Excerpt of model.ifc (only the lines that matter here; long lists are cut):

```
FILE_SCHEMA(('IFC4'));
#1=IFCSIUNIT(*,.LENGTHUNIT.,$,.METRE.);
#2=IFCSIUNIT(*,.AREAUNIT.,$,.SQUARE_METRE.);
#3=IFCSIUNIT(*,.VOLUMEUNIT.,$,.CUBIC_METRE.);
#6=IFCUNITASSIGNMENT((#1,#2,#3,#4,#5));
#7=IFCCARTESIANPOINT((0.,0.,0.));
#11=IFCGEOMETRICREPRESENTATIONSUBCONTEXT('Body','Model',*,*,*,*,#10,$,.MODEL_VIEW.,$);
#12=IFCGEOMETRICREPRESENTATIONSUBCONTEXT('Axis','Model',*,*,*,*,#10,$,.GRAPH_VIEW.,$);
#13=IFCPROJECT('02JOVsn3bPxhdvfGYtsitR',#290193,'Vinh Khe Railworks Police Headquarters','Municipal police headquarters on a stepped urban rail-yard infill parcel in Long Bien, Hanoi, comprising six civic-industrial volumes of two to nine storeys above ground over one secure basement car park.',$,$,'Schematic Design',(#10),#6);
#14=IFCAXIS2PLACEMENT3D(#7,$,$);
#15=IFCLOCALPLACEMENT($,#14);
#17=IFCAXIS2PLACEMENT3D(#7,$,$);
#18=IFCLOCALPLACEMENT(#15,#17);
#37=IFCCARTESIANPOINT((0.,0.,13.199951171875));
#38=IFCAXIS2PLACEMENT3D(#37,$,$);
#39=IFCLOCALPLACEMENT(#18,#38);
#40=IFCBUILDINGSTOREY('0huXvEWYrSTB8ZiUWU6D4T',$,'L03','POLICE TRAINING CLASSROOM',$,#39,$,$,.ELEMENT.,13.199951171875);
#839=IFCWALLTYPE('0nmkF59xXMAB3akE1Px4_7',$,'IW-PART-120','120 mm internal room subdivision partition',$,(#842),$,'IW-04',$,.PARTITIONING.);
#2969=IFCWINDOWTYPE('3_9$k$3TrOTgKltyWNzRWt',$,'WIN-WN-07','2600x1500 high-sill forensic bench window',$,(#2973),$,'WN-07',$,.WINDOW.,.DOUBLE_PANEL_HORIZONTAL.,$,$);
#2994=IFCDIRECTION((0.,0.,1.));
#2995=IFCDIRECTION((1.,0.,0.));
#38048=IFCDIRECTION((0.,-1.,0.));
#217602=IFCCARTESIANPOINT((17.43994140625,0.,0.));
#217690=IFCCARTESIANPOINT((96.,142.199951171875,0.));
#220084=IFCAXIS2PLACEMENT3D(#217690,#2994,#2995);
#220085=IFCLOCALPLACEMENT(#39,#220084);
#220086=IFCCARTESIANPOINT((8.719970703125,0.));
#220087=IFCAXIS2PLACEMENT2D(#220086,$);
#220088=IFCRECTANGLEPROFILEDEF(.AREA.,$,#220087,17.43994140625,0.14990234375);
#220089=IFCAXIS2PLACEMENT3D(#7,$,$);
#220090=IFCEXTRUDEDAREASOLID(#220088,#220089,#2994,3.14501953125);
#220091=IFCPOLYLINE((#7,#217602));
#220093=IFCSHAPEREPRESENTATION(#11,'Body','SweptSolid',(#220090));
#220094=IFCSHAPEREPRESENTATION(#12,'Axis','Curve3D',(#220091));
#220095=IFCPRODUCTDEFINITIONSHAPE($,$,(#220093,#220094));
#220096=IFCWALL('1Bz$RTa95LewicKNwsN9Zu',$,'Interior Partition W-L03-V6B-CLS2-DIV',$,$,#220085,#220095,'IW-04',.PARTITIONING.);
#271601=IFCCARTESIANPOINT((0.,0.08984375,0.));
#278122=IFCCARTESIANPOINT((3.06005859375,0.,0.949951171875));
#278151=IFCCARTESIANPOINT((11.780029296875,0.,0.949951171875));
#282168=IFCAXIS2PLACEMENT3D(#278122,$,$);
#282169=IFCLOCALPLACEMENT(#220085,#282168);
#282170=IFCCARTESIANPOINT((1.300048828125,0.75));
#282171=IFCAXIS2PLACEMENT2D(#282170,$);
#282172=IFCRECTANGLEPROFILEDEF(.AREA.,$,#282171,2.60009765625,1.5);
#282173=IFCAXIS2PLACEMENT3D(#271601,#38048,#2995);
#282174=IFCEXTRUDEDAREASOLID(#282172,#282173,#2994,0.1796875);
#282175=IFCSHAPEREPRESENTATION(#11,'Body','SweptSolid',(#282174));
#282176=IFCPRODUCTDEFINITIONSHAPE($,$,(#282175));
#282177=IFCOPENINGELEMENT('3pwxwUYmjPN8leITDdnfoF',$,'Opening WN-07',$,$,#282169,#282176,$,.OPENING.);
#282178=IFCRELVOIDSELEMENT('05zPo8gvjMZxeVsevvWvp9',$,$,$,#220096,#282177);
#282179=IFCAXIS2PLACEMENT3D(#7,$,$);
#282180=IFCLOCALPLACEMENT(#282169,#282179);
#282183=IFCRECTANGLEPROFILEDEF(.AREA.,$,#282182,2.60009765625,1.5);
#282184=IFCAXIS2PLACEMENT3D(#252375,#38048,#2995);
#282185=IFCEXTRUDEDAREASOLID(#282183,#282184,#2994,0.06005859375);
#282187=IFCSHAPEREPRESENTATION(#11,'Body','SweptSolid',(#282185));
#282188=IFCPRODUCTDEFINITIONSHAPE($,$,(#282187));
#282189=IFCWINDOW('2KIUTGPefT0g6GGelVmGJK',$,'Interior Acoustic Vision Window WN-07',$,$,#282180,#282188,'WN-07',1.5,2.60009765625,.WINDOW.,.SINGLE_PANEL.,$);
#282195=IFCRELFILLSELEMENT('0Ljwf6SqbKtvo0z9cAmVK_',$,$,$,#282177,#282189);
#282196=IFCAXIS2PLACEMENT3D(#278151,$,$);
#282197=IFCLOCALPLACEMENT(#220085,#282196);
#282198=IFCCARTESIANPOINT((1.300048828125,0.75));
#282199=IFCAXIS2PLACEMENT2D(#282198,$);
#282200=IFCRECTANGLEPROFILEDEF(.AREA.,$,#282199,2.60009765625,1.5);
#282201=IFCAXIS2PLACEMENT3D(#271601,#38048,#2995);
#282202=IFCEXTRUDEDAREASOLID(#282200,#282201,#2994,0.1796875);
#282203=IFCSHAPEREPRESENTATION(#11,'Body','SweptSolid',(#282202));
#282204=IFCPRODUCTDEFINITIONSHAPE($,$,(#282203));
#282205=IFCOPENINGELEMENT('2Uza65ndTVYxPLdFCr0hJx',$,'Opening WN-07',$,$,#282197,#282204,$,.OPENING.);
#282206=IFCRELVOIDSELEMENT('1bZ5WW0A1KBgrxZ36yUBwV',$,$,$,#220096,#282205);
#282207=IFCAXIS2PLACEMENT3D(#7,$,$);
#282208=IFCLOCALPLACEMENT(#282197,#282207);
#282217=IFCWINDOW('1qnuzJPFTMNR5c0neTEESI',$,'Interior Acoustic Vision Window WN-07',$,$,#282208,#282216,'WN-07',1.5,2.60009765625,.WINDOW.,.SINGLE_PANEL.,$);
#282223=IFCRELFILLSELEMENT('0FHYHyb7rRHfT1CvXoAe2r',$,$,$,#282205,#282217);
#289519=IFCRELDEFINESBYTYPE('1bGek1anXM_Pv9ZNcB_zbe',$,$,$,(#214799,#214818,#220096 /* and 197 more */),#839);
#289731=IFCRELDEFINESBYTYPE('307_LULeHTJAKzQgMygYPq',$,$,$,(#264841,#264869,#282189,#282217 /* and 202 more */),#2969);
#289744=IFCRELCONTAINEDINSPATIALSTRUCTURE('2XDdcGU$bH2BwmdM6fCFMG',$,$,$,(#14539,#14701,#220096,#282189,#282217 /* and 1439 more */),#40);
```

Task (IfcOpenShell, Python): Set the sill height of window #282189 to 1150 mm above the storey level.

```python
import numpy as np
import ifcopenshell
import ifcopenshell.api.geometry
import ifcopenshell.geom
import ifcopenshell.util.element
import ifcopenshell.util.placement
import ifcopenshell.util.shape
import ifcopenshell.util.unit

model = ifcopenshell.open("model.ifc")
unit_scale = ifcopenshell.util.unit.calculate_unit_scale(model)

window = model.by_guid("2KIUTGPefT0g6GGelVmGJK")
opening = window.FillsVoids[0].RelatingOpeningElement
storey = ifcopenshell.util.element.get_container(window, ifc_class="IfcBuildingStorey")
level = ifcopenshell.util.placement.get_local_placement(storey.ObjectPlacement)[2, 3]

# The opening's origin need not be at the sill, so measure its lowest point.
shape = ifcopenshell.geom.create_shape(ifcopenshell.geom.settings(), opening)
bottom = ifcopenshell.util.shape.get_shape_bottom_elevation(shape, shape.geometry) / unit_scale
dz = level + 1.15 / unit_scale - bottom

shift = np.array([0.0, 0.0, dz])
# The window is placed relative to its opening, so it follows when the opening moves.
matrix = ifcopenshell.util.placement.get_local_placement(opening.ObjectPlacement)
matrix[:3, 3] += shift
ifcopenshell.api.geometry.edit_object_placement(
    model, product=opening, matrix=matrix, is_si=False, should_transform_children=True
)

print(f"moved by {dz * unit_scale:+.3f} m")

model.write("model_rev.ifc")
```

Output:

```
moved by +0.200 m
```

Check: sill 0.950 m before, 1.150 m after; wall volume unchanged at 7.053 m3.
